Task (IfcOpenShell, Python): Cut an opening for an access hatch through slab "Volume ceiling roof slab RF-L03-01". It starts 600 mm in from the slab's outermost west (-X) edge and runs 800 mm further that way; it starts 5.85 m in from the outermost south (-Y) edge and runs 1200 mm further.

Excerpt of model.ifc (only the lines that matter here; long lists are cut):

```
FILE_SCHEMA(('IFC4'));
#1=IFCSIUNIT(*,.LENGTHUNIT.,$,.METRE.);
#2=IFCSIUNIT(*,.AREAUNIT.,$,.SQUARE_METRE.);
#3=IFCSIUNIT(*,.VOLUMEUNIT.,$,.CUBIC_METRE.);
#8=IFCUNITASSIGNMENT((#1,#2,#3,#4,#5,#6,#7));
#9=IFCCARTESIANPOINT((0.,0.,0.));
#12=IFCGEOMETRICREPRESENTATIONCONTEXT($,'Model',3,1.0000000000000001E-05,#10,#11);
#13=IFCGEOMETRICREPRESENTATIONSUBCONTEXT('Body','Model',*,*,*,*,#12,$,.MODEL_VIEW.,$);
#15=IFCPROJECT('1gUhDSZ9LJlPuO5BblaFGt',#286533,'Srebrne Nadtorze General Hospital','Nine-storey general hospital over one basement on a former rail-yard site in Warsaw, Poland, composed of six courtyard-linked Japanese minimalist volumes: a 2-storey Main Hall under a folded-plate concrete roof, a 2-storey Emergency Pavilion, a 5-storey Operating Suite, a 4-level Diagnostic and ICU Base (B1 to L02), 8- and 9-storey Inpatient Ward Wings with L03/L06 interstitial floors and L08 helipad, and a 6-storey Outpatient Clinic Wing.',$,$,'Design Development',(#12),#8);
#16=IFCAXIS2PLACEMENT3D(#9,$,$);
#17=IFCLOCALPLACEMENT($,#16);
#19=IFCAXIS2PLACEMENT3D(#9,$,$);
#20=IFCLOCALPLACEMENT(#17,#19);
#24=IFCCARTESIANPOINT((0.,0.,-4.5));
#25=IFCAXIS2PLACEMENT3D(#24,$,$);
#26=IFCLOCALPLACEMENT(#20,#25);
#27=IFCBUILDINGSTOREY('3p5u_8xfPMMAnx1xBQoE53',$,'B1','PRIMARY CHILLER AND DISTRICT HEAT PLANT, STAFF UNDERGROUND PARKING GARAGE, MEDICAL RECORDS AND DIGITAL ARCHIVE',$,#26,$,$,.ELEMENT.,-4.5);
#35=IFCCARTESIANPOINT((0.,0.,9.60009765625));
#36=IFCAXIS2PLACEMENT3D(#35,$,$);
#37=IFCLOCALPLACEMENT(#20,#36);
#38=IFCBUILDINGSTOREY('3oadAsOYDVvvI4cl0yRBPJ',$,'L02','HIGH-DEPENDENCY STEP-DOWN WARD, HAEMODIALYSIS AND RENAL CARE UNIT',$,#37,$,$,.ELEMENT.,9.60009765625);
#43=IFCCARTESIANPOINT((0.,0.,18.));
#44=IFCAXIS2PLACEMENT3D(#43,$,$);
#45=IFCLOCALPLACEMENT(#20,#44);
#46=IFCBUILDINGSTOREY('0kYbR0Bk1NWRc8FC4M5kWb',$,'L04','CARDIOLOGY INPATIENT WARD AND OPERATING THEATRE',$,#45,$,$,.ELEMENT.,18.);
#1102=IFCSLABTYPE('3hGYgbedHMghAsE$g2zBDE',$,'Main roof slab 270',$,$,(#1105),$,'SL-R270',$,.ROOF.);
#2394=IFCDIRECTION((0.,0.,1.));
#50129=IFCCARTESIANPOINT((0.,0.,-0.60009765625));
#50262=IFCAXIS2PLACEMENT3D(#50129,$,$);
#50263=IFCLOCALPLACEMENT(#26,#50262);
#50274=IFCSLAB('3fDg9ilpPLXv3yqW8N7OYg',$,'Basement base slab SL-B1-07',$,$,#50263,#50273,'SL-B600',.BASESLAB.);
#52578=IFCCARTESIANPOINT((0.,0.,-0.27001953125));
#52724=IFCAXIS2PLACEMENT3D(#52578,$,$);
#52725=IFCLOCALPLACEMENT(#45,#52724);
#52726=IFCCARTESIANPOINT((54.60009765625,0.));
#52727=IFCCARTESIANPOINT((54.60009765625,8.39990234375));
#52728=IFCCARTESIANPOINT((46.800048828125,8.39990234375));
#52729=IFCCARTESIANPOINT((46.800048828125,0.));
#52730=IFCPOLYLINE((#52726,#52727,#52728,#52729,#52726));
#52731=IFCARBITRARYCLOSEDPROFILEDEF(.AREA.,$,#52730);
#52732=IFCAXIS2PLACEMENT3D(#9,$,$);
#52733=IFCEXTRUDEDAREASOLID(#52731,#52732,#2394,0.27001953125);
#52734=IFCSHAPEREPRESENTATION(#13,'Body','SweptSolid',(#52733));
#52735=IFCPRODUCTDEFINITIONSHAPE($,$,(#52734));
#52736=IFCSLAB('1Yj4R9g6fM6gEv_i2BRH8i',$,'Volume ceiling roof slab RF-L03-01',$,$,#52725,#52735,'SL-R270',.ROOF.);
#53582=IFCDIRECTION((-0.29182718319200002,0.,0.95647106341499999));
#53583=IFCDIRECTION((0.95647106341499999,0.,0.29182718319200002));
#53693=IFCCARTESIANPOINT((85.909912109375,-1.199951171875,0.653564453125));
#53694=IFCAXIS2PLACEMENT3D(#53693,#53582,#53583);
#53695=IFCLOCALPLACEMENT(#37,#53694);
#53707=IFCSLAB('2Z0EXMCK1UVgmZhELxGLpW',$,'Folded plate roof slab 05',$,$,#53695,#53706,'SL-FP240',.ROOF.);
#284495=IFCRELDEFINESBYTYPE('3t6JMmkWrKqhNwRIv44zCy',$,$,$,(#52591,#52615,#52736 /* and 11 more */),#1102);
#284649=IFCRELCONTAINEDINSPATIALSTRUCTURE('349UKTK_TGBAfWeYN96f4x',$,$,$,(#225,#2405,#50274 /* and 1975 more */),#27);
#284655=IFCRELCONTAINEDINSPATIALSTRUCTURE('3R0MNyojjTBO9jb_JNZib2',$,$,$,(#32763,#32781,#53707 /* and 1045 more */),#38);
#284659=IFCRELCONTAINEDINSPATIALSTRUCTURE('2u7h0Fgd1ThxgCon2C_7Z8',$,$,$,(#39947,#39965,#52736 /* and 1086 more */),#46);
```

```python
import numpy as np
import ifcopenshell
import ifcopenshell.api.feature
import ifcopenshell.api.geometry
import ifcopenshell.api.root
import ifcopenshell.geom
import ifcopenshell.util.placement
import ifcopenshell.util.representation
import ifcopenshell.util.shape
import ifcopenshell.util.unit

model = ifcopenshell.open("model.ifc")
unit_scale = ifcopenshell.util.unit.calculate_unit_scale(model)
settings = ifcopenshell.geom.settings()


def volume(element):
    """Net volume in cubic metres, openings subtracted."""
    shape = ifcopenshell.geom.create_shape(settings, element)
    return ifcopenshell.util.shape.get_volume(shape.geometry)


slab = model.by_guid("1Yj4R9g6fM6gEv_i2BRH8i")
before = volume(slab)

# Extent in the slab's own axes, in metres. The edges named are its -X and -Y sides.
slab_shape = ifcopenshell.geom.create_shape(settings, slab)
vertices = ifcopenshell.util.shape.get_vertices(slab_shape.geometry)
x_min, y_min, bottom = vertices.min(axis=0)
top = vertices[:, 2].max()

opening = ifcopenshell.api.root.create_entity(model, ifc_class="IfcOpeningElement", name="Access hatch opening", predefined_type="OPENING")
context = ifcopenshell.util.representation.get_context(model, "Model", "Body", "MODEL_VIEW")
width, depth = 0.8, 1.2
outline = [(0.0, 0.0), (width, 0.0), (width, depth), (0.0, depth), (0.0, 0.0)]
# Overshoot both faces by 50 mm so the cut is clean.
shape = ifcopenshell.api.geometry.add_slab_representation(
    model, context=context, depth=top - bottom + 0.1, polyline=outline
)
ifcopenshell.api.geometry.assign_representation(model, product=opening, representation=shape)

matrix = ifcopenshell.util.placement.get_local_placement(slab.ObjectPlacement)
matrix[:, 3] = matrix @ np.append(np.array([x_min + 0.6, y_min + 5.85, bottom - 0.05]) / unit_scale, 1.0)
ifcopenshell.api.geometry.edit_object_placement(model, product=opening, matrix=matrix, is_si=False)
ifcopenshell.api.feature.add_feature(model, feature=opening, element=slab)

after = volume(slab)

print(f"slab volume {before:.3f} -> {after:.3f} m3")

model.write("model_rev.ifc")
```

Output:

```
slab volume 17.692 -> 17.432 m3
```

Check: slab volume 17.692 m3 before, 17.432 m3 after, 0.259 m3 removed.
